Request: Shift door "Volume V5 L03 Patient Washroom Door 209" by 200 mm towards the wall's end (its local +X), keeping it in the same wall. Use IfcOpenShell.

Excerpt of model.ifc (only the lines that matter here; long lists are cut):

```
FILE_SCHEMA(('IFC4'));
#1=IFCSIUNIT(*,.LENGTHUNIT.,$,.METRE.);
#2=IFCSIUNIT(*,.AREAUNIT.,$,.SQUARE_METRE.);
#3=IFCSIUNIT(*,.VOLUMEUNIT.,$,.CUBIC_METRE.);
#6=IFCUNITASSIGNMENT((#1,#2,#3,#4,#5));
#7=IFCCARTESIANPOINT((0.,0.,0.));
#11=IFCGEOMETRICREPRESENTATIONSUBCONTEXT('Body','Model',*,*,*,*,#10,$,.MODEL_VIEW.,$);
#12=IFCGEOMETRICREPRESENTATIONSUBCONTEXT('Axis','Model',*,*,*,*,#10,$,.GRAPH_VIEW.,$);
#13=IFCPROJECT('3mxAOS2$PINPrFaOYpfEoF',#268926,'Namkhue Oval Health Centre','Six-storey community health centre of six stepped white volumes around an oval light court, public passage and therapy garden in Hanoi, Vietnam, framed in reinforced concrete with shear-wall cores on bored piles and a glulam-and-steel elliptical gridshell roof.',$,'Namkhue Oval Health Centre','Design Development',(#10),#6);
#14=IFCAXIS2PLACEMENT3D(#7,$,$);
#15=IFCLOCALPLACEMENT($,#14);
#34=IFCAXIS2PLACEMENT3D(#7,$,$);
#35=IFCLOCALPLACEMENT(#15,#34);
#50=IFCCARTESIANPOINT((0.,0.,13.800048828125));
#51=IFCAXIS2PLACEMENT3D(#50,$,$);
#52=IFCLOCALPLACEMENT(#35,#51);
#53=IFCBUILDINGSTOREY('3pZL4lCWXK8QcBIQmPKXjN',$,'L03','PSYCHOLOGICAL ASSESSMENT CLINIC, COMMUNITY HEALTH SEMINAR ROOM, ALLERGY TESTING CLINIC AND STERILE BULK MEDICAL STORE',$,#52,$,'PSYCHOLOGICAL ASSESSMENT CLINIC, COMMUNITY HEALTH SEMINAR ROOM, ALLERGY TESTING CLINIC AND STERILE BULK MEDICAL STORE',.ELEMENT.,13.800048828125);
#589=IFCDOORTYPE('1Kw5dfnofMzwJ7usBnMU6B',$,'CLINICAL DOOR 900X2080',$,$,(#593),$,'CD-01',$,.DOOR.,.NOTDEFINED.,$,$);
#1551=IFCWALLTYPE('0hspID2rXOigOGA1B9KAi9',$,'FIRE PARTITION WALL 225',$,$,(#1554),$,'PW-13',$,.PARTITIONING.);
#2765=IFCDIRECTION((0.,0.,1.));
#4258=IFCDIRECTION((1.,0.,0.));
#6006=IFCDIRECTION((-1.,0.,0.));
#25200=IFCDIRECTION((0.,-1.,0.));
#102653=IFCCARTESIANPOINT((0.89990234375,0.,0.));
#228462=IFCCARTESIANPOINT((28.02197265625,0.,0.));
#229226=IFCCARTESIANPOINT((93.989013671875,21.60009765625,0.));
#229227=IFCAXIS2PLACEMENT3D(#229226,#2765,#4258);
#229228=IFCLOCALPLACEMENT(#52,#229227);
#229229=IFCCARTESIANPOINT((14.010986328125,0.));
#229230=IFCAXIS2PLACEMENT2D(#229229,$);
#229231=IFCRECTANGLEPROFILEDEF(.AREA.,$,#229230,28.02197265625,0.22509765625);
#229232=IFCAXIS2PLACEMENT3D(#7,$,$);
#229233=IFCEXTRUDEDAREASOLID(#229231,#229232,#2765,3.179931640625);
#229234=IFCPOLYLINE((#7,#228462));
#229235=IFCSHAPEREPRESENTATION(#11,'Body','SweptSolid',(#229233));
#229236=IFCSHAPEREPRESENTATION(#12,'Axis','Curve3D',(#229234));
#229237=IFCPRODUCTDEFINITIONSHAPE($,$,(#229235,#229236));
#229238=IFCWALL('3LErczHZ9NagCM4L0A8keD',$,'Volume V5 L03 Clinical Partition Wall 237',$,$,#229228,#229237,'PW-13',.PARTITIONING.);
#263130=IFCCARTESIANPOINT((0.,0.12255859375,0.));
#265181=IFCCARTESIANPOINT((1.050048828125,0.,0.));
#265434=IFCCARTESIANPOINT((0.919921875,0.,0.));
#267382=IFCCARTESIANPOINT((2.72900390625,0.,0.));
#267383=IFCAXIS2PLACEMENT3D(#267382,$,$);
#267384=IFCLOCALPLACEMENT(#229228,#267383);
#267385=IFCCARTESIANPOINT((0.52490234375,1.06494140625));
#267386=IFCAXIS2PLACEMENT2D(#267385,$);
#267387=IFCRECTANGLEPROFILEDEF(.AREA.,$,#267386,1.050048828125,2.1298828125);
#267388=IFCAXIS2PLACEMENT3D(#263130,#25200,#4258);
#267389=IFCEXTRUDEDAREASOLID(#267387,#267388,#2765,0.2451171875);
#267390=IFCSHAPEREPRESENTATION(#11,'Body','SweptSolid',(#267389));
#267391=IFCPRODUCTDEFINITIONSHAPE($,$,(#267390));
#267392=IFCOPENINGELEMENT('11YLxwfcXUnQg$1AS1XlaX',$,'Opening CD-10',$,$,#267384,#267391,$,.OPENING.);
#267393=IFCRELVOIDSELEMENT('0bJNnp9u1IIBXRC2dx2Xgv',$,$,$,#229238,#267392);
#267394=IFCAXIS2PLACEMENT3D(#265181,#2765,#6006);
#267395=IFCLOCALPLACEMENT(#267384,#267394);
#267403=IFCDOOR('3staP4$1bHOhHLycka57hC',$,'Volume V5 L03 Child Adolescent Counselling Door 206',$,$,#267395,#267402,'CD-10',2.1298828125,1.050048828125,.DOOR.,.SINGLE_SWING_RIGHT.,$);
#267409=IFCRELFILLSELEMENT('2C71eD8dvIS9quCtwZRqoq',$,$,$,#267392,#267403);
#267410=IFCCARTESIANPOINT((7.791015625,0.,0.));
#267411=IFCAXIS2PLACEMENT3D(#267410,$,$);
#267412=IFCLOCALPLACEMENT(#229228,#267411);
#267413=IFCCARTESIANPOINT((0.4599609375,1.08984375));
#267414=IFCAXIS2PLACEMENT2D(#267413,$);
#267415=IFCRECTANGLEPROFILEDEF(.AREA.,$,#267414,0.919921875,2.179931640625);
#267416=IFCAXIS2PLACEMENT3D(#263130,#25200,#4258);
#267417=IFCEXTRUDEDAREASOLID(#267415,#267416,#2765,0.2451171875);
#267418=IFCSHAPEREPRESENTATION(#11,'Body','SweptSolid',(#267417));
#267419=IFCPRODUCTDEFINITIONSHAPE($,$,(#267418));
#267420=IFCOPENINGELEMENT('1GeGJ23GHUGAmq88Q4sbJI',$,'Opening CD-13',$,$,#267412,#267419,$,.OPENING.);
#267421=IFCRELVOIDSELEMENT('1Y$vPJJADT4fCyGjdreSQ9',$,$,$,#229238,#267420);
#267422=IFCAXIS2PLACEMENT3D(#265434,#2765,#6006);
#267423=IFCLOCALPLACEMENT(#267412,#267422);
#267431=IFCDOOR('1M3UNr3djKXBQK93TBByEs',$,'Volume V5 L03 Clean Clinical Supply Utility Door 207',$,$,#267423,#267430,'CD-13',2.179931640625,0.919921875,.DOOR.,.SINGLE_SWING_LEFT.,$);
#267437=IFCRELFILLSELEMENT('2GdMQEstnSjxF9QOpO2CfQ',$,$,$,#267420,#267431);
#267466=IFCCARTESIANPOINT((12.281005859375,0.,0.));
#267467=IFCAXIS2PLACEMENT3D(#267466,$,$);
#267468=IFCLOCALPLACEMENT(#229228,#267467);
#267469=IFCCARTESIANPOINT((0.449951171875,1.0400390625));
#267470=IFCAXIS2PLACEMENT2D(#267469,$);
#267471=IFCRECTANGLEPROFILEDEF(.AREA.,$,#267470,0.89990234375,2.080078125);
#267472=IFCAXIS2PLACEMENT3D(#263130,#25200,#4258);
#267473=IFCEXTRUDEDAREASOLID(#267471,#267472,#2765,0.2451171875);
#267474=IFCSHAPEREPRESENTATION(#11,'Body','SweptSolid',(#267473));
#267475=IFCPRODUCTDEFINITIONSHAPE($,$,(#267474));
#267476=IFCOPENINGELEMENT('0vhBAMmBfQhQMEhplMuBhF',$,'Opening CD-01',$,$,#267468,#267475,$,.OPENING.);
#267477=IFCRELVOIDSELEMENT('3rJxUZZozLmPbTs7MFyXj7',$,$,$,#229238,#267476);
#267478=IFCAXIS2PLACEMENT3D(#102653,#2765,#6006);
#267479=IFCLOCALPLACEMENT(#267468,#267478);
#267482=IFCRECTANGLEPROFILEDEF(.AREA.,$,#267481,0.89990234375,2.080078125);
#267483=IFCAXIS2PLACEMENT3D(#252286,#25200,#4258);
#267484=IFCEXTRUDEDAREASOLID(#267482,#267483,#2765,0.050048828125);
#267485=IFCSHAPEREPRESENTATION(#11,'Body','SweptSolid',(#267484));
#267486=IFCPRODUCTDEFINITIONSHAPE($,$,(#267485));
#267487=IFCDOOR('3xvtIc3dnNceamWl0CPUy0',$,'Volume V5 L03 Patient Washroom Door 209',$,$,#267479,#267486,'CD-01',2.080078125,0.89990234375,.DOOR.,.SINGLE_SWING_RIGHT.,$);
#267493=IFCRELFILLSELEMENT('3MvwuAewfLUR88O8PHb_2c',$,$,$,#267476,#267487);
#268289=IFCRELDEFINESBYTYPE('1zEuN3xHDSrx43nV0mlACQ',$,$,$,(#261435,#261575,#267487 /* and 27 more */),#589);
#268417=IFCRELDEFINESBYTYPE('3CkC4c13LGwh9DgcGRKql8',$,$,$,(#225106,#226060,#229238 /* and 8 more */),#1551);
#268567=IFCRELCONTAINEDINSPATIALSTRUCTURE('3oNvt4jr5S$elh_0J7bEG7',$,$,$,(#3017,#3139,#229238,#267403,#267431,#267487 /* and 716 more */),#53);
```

```python
import ifcopenshell
import ifcopenshell.api.geometry
import ifcopenshell.util.placement
import ifcopenshell.util.unit

model = ifcopenshell.open("model.ifc")
unit_scale = ifcopenshell.util.unit.calculate_unit_scale(model)

door = model.by_guid("3xvtIc3dnNceamWl0CPUy0")
opening = door.FillsVoids[0].RelatingOpeningElement
wall = opening.VoidsElements[0].RelatingBuildingElement

wall_matrix = ifcopenshell.util.placement.get_local_placement(wall.ObjectPlacement)
shift = wall_matrix[:3, 0] * 0.2 / unit_scale
before = ifcopenshell.util.placement.get_local_placement(door.ObjectPlacement)[:3, 3].copy()

# The door is placed relative to its opening, so it follows when the opening moves.
matrix = ifcopenshell.util.placement.get_local_placement(opening.ObjectPlacement)
matrix[:3, 3] += shift
ifcopenshell.api.geometry.edit_object_placement(
    model, product=opening, matrix=matrix, is_si=False, should_transform_children=True
)

after = ifcopenshell.util.placement.get_local_placement(door.ObjectPlacement)[:3, 3]
print("door moved by", (after - before).round(3) + 0.0)

model.write("model-out.ifc")
```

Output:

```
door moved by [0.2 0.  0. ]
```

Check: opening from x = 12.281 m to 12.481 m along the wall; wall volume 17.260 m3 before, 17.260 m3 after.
